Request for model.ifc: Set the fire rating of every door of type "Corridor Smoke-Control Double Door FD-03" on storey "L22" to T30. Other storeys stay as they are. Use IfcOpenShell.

First a look at what the model holds.

```python
import ifcopenshell
import ifcopenshell.util.element

model = ifcopenshell.open("model.ifc")
print(model.schema)
storey = next(s for s in model.by_type("IfcBuildingStorey") if s.Name == "L22")
doors = [e for e in ifcopenshell.util.element.get_decomposition(storey) if e.is_a("IfcDoor")]
seen = {}
for e in doors:
    element_type = ifcopenshell.util.element.get_type(e)
    key = (element_type.Name if element_type != e and element_type else None, ifcopenshell.util.element.get_pset(e, "Pset_DoorCommon", "FireRating"))
    seen[key] = seen.get(key, 0) + 1
for (name, value), count in sorted(seen.items(), key=str):
    print(count, "x", name, "|", value)
```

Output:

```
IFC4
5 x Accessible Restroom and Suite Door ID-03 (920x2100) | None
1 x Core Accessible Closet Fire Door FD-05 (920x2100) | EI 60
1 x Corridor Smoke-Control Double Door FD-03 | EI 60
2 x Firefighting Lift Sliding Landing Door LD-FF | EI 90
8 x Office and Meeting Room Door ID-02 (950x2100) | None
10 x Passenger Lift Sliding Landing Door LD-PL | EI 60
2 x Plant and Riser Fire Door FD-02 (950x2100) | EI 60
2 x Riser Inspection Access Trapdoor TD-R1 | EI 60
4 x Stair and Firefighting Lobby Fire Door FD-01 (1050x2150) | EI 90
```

```python
import ifcopenshell
import ifcopenshell.api.pset
import ifcopenshell.util.element

model = ifcopenshell.open("model.ifc")

storey = next(s for s in model.by_type("IfcBuildingStorey") if s.Name == "L22")
doors = [e for e in ifcopenshell.util.element.get_decomposition(storey) if e.is_a("IfcDoor")]

count = 0
for e in doors:
    element_type = ifcopenshell.util.element.get_type(e)
    if element_type in (None, e) or element_type.Name != "Corridor Smoke-Control Double Door FD-03":
        continue
    found = ifcopenshell.util.element.get_pset(e, "Pset_DoorCommon", should_inherit=False)
    if found:
        pset = model.by_id(found["id"])
        if len(ifcopenshell.util.element.get_elements_by_pset(pset)) > 1:
            pset = ifcopenshell.api.pset.unshare_pset(model, products=[e], pset=pset)[0]
    else:
        pset = ifcopenshell.api.pset.add_pset(model, product=e, name="Pset_DoorCommon")
    ifcopenshell.api.pset.edit_pset(model, pset=pset, properties={"FireRating": "T30"})
    count += 1

print(count, "doors updated")

model.write("model_rev.ifc")
```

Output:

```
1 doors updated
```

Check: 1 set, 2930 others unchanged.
